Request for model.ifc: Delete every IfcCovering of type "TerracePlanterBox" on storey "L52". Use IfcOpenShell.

First a look at what the model holds.

```python
import ifcopenshell
import ifcopenshell.util.element

model = ifcopenshell.open("model.ifc")
print(model.schema)
storey = next(s for s in model.by_type("IfcBuildingStorey") if s.Name == "L52")
coverings = [e for e in ifcopenshell.util.element.get_decomposition(storey) if e.is_a("IfcCovering")]
seen = {}
for e in coverings:
    element_type = ifcopenshell.util.element.get_type(e)
    name = element_type.Name if element_type not in (None, e) else None
    seen[name] = seen.get(name, 0) + 1
for name, count in sorted(seen.items(), key=str):
    print(count, "x", name)
```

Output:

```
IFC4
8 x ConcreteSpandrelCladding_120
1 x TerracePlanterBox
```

```python
import ifcopenshell
import ifcopenshell.api.root
import ifcopenshell.util.element

model = ifcopenshell.open("model.ifc")

storey = next(s for s in model.by_type("IfcBuildingStorey") if s.Name == "L52")
coverings = [e for e in ifcopenshell.util.element.get_decomposition(storey) if e.is_a("IfcCovering")]
targets = [e for e in coverings if (t := ifcopenshell.util.element.get_type(e)) not in (None, e) and t.Name == "TerracePlanterBox"]

for e in targets:
    ifcopenshell.api.root.remove_product(model, product=e)
print(len(targets), "removed")

model.write("model_updated.ifc")
```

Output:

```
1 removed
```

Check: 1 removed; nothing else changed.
